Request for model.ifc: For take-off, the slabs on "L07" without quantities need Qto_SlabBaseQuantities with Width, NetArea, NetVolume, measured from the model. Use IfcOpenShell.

First a look at what the model holds.

```python
import ifcopenshell
import ifcopenshell.util.element
import ifcopenshell.util.unit

model = ifcopenshell.open("model.ifc")
print(model.schema)
for unit_type in ("LENGTHUNIT", "AREAUNIT", "VOLUMEUNIT"):
    print(unit_type, ifcopenshell.util.unit.calculate_unit_scale(model, unit_type))
storey = next(s for s in model.by_type("IfcBuildingStorey") if s.Name == "L07")
slabs = [e for e in ifcopenshell.util.element.get_decomposition(storey) if e.is_a("IfcSlab")]
for e in sorted(slabs, key=lambda e: e.id()):
    print(e.id(), e.is_a(), e.Name, list(ifcopenshell.util.element.get_psets(e, qtos_only=True)), sep=" | ")
```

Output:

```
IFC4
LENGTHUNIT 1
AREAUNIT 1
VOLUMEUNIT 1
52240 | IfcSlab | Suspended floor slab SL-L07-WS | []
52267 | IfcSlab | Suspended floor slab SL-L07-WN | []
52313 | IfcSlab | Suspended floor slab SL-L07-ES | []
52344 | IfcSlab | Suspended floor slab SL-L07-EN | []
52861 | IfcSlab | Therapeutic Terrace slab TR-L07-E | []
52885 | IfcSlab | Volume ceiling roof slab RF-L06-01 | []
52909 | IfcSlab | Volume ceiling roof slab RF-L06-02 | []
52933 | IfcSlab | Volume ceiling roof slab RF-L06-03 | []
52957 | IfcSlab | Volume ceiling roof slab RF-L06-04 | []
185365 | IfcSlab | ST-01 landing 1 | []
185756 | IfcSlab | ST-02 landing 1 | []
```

```python
import ifcopenshell
import ifcopenshell.api.pset
import ifcopenshell.geom
import ifcopenshell.util.element
import ifcopenshell.util.shape
import ifcopenshell.util.unit

model = ifcopenshell.open("model.ifc")
unit_scale = ifcopenshell.util.unit.calculate_unit_scale(model)
area_scale = ifcopenshell.util.unit.calculate_unit_scale(model, "AREAUNIT")
volume_scale = ifcopenshell.util.unit.calculate_unit_scale(model, "VOLUMEUNIT")
settings = ifcopenshell.geom.settings()

storey = next(s for s in model.by_type("IfcBuildingStorey") if s.Name == "L07")
slabs = [e for e in ifcopenshell.util.element.get_decomposition(storey) if e.is_a("IfcSlab")]

for e in sorted(slabs, key=lambda e: e.id()):
    if ifcopenshell.util.element.get_psets(e, qtos_only=True, should_inherit=False):
        continue
    # Geometry comes back in metres, in the element's own axes.
    shape = ifcopenshell.geom.create_shape(settings, e)
    values = {
        "Width": ifcopenshell.util.shape.get_z(shape.geometry) / unit_scale,
        "NetArea": ifcopenshell.util.shape.get_footprint_area(shape.geometry) / area_scale,
        "NetVolume": ifcopenshell.util.shape.get_volume(shape.geometry) / volume_scale,
    }
    qto = ifcopenshell.api.pset.add_qto(model, product=e, name="Qto_SlabBaseQuantities")
    ifcopenshell.api.pset.edit_qto(model, qto=qto, properties=values)
    print(e.id(), {k: round(v, 3) for k, v in values.items()})

model.write("model-out.ifc")
```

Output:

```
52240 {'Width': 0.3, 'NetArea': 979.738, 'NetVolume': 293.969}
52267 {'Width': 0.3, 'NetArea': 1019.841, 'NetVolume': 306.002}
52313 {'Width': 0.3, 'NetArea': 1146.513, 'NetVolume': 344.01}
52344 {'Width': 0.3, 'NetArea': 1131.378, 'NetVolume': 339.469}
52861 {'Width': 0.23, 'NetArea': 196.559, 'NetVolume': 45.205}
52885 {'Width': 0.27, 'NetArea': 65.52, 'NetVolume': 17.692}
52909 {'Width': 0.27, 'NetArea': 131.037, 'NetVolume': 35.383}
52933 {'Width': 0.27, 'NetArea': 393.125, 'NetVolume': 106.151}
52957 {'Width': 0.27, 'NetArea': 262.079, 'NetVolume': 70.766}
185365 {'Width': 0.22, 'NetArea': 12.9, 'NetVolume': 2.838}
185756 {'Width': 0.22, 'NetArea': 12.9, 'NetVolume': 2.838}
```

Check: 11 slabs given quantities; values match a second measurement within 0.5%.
